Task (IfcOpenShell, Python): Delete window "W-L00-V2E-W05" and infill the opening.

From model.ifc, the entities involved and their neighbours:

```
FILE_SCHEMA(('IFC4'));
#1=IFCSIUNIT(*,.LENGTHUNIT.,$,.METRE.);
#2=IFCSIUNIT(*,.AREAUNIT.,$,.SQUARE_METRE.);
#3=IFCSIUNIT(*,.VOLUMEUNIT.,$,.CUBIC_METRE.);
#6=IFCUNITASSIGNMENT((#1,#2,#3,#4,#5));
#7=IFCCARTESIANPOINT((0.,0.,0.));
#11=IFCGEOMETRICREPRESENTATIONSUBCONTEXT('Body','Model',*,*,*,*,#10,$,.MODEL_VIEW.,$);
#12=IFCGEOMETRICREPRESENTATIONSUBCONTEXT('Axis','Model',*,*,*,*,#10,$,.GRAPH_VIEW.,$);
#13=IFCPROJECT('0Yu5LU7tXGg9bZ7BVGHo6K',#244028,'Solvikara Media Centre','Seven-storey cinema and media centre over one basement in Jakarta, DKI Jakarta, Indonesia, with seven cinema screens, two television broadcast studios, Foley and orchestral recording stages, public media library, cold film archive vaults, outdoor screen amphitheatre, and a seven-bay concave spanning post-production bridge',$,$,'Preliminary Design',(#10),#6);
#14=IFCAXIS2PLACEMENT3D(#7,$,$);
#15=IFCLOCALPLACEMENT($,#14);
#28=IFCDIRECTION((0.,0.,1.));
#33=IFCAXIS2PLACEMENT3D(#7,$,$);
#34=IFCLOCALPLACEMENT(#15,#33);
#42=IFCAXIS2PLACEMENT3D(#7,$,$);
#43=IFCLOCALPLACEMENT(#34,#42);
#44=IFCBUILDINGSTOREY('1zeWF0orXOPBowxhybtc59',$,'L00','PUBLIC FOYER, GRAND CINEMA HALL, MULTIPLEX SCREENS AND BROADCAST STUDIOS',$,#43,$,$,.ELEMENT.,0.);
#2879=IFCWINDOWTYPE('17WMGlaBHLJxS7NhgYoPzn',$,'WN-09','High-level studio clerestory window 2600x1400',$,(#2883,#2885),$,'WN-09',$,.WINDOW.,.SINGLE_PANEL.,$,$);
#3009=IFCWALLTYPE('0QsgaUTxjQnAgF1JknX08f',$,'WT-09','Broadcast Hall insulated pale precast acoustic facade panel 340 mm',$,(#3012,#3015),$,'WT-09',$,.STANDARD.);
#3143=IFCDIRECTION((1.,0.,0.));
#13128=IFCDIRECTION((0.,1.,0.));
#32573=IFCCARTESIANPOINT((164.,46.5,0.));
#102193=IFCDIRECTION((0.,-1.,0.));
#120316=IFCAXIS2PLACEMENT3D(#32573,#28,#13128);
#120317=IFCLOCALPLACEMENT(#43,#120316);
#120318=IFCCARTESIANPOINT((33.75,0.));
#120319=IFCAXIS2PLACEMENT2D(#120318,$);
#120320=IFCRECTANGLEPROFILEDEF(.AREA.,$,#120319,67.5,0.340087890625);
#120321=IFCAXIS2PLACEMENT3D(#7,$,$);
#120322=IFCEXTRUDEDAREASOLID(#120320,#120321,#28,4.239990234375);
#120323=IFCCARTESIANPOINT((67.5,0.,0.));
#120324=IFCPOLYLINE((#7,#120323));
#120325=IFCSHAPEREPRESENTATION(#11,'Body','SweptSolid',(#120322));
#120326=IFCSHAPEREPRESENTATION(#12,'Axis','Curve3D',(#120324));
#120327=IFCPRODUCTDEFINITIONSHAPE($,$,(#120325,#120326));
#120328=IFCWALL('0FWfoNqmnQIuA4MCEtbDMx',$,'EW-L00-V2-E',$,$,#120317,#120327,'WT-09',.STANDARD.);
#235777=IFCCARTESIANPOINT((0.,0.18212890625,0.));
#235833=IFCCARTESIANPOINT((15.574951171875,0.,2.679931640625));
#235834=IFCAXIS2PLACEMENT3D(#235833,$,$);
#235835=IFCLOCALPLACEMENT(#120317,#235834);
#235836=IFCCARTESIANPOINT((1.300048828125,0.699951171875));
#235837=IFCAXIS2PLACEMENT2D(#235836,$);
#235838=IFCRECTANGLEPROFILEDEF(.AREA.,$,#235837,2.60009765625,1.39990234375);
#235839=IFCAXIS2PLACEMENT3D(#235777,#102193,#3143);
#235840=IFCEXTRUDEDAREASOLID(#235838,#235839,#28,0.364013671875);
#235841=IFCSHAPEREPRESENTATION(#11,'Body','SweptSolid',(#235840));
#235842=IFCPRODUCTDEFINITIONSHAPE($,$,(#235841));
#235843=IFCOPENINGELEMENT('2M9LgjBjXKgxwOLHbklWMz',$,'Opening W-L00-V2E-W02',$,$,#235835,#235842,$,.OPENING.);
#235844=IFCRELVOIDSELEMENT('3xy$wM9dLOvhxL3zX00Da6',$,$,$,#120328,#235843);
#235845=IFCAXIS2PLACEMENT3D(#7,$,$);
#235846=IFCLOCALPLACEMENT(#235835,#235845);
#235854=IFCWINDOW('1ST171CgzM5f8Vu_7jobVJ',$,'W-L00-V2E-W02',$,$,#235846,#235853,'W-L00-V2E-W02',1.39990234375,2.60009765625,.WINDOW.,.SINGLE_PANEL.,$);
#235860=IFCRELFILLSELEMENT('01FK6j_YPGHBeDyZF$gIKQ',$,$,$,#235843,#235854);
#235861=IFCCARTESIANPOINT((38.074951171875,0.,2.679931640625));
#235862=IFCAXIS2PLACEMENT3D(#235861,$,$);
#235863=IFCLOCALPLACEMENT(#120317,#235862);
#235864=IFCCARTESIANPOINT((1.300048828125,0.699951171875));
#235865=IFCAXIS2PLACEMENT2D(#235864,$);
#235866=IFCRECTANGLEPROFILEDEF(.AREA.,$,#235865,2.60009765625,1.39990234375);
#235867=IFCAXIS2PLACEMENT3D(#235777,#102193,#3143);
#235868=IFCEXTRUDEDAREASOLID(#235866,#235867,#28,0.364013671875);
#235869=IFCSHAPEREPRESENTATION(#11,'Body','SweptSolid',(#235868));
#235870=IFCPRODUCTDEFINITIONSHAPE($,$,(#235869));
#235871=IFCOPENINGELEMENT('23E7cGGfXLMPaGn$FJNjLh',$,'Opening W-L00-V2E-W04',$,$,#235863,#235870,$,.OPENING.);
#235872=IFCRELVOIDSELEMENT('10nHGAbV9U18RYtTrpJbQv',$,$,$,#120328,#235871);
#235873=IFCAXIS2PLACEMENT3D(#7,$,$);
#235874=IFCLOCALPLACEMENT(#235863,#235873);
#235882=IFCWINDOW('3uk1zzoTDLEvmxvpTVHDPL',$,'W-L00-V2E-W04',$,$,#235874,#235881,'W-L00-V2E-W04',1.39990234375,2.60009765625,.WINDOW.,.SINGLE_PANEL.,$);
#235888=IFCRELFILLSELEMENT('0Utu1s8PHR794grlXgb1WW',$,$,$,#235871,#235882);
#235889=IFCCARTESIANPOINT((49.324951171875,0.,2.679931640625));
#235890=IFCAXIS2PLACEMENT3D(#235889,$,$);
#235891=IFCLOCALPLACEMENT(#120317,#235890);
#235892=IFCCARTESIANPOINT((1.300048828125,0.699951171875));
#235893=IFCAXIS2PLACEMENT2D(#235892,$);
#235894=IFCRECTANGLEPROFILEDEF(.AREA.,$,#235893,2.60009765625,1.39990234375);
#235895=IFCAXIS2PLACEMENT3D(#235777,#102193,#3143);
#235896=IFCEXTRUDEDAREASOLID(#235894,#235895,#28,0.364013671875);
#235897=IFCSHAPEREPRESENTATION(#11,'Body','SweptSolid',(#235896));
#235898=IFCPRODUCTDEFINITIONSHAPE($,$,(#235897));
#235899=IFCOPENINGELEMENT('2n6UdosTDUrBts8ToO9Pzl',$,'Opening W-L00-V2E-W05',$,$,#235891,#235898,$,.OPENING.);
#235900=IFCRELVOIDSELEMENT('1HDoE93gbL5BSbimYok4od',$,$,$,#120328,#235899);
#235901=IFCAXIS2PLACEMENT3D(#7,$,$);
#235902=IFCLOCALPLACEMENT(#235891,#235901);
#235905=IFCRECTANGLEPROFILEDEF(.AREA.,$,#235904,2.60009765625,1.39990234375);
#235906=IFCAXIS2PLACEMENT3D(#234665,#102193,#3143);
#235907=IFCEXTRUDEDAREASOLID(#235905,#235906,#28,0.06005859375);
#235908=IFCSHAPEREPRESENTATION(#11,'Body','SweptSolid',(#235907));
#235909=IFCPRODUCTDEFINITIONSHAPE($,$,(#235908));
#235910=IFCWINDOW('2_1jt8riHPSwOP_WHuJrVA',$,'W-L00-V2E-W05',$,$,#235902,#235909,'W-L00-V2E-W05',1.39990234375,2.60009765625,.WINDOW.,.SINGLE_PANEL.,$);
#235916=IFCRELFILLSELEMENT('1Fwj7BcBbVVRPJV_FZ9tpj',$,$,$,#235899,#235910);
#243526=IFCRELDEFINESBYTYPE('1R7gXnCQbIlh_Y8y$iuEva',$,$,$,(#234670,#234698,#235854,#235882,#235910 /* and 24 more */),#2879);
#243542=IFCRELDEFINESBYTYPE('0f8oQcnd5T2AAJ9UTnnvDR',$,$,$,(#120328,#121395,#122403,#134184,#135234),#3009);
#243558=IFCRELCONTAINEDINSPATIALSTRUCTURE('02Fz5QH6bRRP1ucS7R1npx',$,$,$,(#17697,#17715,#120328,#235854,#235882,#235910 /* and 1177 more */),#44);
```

```python
import ifcopenshell
import ifcopenshell.api.feature
import ifcopenshell.api.root
import ifcopenshell.geom
import ifcopenshell.util.shape

model = ifcopenshell.open("model.ifc")
settings = ifcopenshell.geom.settings()


def volume(element):
    """Net volume in cubic metres, openings subtracted."""
    shape = ifcopenshell.geom.create_shape(settings, element)
    return ifcopenshell.util.shape.get_volume(shape.geometry)


window = model.by_id(235910)
opening = window.FillsVoids[0].RelatingOpeningElement
wall = opening.VoidsElements[0].RelatingBuildingElement
before = volume(wall)

ifcopenshell.api.root.remove_product(model, product=window)
ifcopenshell.api.feature.remove_feature(model, feature=opening)

after = volume(wall)

print(f"wall volume {before:.3f} -> {after:.3f} m3")

model.write("model_updated.ifc")
```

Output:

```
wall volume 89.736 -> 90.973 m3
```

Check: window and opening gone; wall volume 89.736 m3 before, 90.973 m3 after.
